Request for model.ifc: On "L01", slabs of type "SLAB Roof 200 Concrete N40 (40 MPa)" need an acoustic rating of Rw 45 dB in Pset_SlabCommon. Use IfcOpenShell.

First a look at what the model holds.

```python
import ifcopenshell
import ifcopenshell.util.element

model = ifcopenshell.open("model.ifc")
print(model.schema)
storey = next(s for s in model.by_type("IfcBuildingStorey") if s.Name == "L01")
slabs = [e for e in ifcopenshell.util.element.get_decomposition(storey) if e.is_a("IfcSlab")]
seen = {}
for e in slabs:
    element_type = ifcopenshell.util.element.get_type(e)
    key = (element_type.Name if element_type != e and element_type else None, ifcopenshell.util.element.get_pset(e, "Pset_SlabCommon", "AcousticRating"))
    seen[key] = seen.get(key, 0) + 1
for (name, value), count in sorted(seen.items(), key=str):
    print(count, "x", name, "|", value)
```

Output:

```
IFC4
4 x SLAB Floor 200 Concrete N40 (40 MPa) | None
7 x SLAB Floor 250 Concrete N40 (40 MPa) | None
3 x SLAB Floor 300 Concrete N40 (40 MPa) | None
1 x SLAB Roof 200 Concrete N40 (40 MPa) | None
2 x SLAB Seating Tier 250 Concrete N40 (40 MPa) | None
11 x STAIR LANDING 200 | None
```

```python
import ifcopenshell
import ifcopenshell.api.pset
import ifcopenshell.util.element

model = ifcopenshell.open("model.ifc")

storey = next(s for s in model.by_type("IfcBuildingStorey") if s.Name == "L01")
slabs = [e for e in ifcopenshell.util.element.get_decomposition(storey) if e.is_a("IfcSlab")]

count = 0
for e in slabs:
    element_type = ifcopenshell.util.element.get_type(e)
    if element_type in (None, e) or element_type.Name != "SLAB Roof 200 Concrete N40 (40 MPa)":
        continue
    # add_pset returns the element's existing set when there is one.
    pset = ifcopenshell.api.pset.add_pset(model, product=e, name="Pset_SlabCommon")
    ifcopenshell.api.pset.edit_pset(model, pset=pset, properties={"AcousticRating": "Rw 45 dB"})
    count += 1

print(count, "slabs updated")

model.write("model_rev.ifc")
```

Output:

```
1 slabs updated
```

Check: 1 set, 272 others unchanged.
